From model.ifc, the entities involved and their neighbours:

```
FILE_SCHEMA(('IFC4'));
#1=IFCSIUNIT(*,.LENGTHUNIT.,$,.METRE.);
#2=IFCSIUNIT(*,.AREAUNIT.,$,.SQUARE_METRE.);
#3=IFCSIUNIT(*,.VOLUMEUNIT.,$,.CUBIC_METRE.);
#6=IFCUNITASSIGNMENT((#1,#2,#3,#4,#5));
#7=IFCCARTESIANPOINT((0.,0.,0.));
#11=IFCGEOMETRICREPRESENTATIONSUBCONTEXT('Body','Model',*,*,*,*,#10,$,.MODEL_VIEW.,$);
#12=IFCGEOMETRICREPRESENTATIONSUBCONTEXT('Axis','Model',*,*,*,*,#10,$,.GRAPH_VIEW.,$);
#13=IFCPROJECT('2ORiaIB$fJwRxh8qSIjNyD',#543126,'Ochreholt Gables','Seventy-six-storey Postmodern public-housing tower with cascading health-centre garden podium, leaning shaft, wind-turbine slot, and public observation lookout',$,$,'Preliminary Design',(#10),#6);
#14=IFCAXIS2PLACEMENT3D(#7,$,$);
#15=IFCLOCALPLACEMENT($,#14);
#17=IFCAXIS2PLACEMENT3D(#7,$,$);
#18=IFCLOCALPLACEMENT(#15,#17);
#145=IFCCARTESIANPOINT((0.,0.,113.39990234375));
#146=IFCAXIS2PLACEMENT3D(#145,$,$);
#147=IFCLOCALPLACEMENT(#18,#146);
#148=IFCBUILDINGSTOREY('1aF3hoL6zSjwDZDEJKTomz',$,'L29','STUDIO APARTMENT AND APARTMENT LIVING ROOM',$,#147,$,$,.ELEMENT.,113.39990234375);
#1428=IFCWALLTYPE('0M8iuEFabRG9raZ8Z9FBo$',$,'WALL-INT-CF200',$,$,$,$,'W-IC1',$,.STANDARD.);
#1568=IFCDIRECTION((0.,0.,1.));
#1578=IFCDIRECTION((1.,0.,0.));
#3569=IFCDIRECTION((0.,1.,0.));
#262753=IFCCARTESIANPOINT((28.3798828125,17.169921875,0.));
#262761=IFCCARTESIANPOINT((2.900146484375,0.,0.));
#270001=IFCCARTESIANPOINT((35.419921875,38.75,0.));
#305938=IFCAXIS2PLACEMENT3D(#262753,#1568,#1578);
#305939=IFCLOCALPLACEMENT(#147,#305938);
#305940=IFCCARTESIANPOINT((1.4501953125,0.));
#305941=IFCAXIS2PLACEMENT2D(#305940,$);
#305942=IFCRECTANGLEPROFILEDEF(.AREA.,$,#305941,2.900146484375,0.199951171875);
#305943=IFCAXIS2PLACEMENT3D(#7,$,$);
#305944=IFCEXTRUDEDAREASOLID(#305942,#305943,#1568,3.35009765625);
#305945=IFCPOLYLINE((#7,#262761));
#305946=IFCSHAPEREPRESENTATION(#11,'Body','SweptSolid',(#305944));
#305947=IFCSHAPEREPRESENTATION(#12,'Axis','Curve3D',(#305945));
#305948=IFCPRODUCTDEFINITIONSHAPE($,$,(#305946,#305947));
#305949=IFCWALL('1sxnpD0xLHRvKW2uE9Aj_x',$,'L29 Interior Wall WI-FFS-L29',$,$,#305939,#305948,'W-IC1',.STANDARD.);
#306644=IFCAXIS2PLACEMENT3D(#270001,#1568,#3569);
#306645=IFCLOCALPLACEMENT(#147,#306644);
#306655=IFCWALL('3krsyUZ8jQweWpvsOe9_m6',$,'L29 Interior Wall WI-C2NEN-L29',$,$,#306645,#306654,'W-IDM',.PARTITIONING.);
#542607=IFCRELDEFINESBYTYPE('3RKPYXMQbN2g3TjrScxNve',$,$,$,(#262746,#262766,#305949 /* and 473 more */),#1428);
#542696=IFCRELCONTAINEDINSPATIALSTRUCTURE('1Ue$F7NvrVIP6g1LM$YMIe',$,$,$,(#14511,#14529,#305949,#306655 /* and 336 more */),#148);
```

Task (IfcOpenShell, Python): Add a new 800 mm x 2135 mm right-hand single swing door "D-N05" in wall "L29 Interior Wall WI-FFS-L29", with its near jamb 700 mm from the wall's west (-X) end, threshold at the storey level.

```python
import numpy as np
import ifcopenshell
import ifcopenshell.api.feature
import ifcopenshell.api.geometry
import ifcopenshell.api.root
import ifcopenshell.api.spatial
import ifcopenshell.geom
import ifcopenshell.util.element
import ifcopenshell.util.placement
import ifcopenshell.util.representation
import ifcopenshell.util.shape
import ifcopenshell.util.unit

model = ifcopenshell.open("model.ifc")
unit_scale = ifcopenshell.util.unit.calculate_unit_scale(model)
settings = ifcopenshell.geom.settings()


def volume(element):
    """Net volume in cubic metres, openings subtracted."""
    shape = ifcopenshell.geom.create_shape(settings, element)
    return ifcopenshell.util.shape.get_volume(shape.geometry)


wall = model.by_guid("1sxnpD0xLHRvKW2uE9Aj_x")
storey = ifcopenshell.util.element.get_container(wall, ifc_class="IfcBuildingStorey")
context = ifcopenshell.util.representation.get_context(model, "Model", "Body", "MODEL_VIEW")
before = volume(wall)

width, height, from_end, sill = 0.8, 2.135, 0.7, 0.0  # metres

# The wall runs along its own X axis, and the end named is its -X end.
wall_shape = ifcopenshell.geom.create_shape(settings, wall)
x, y, z = ifcopenshell.util.shape.get_vertices(wall_shape.geometry).T
start = x.min() + from_end
face, thickness = float(y.min()), float(y.max() - y.min())
wall_matrix = ifcopenshell.util.placement.get_local_placement(wall.ObjectPlacement)
level = ifcopenshell.util.placement.get_local_placement(storey.ObjectPlacement)[2, 3]


def in_wall(x, y):
    """Placement at x, y metres in the wall's axes, at sill height."""
    matrix = wall_matrix.copy()
    matrix[:, 3] = wall_matrix @ np.array([x / unit_scale, y / unit_scale, 0.0, 1.0])
    matrix[2, 3] = level + sill / unit_scale
    return matrix


# Opening: a box that overshoots both wall faces by 50 mm.
opening = ifcopenshell.api.root.create_entity(model, ifc_class="IfcOpeningElement", predefined_type="OPENING")
box = ifcopenshell.api.geometry.add_wall_representation(
    model, context=context, length=width, height=height, thickness=thickness + 0.1
)
ifcopenshell.api.geometry.assign_representation(model, product=opening, representation=box)
ifcopenshell.api.geometry.edit_object_placement(model, product=opening, matrix=in_wall(start, face - 0.05), is_si=False)
ifcopenshell.api.feature.add_feature(model, feature=opening, element=wall)

door = ifcopenshell.api.root.create_entity(model, ifc_class="IfcDoor", name="D-N05", predefined_type="DOOR")
door.OverallWidth, door.OverallHeight = width / unit_scale, height / unit_scale
door.OperationType = "SINGLE_SWING_RIGHT"
body = ifcopenshell.api.geometry.add_door_representation(
    model,
    context=context,
    overall_width=door.OverallWidth,
    overall_height=door.OverallHeight,
    operation_type="SINGLE_SWING_RIGHT",
    lining_properties={"LiningDepth": thickness / unit_scale, "ThresholdDepth": thickness / unit_scale},
)
ifcopenshell.api.geometry.assign_representation(model, product=door, representation=body)
ifcopenshell.api.spatial.assign_container(model, products=[door], relating_structure=storey)
ifcopenshell.api.feature.add_filling(model, opening=opening, element=door)

# The lining spans the wall, so the door starts at the wall face.
ifcopenshell.api.geometry.edit_object_placement(model, product=door, matrix=in_wall(start, face), is_si=False)

after = volume(wall)

print(f"wall volume {before:.3f} -> {after:.3f} m3")

model.write("model_edited.ifc")
```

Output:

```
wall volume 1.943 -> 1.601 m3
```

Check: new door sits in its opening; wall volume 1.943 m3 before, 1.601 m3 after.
